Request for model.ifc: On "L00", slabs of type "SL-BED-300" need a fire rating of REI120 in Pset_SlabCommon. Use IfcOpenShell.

First a look at what the model holds.

```python
import ifcopenshell
import ifcopenshell.util.element

model = ifcopenshell.open("model.ifc")
print(model.schema)
storey = next(s for s in model.by_type("IfcBuildingStorey") if s.Name == "L00")
slabs = [e for e in ifcopenshell.util.element.get_decomposition(storey) if e.is_a("IfcSlab")]
seen = {}
for e in slabs:
    element_type = ifcopenshell.util.element.get_type(e)
    key = (element_type.Name if element_type != e and element_type else None, ifcopenshell.util.element.get_pset(e, "Pset_SlabCommon", "FireRating"))
    seen[key] = seen.get(key, 0) + 1
for (name, value), count in sorted(seen.items(), key=str):
    print(count, "x", name, "|", value)
```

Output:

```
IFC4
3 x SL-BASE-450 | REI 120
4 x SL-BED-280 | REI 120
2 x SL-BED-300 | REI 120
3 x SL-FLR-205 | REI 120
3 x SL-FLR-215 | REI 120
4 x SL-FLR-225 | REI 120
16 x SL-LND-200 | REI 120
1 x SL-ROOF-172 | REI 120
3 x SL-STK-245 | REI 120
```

```python
import ifcopenshell
import ifcopenshell.api.pset
import ifcopenshell.util.element

model = ifcopenshell.open("model.ifc")

storey = next(s for s in model.by_type("IfcBuildingStorey") if s.Name == "L00")
slabs = [e for e in ifcopenshell.util.element.get_decomposition(storey) if e.is_a("IfcSlab")]

count = 0
for e in slabs:
    element_type = ifcopenshell.util.element.get_type(e)
    if element_type in (None, e) or element_type.Name != "SL-BED-300":
        continue
    # add_pset returns the element's existing set when there is one.
    pset = ifcopenshell.api.pset.add_pset(model, product=e, name="Pset_SlabCommon")
    ifcopenshell.api.pset.edit_pset(model, pset=pset, properties={"FireRating": "REI120"})
    count += 1

print(count, "slabs updated")

model.write("model_edited.ifc")
```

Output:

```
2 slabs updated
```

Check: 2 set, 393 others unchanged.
